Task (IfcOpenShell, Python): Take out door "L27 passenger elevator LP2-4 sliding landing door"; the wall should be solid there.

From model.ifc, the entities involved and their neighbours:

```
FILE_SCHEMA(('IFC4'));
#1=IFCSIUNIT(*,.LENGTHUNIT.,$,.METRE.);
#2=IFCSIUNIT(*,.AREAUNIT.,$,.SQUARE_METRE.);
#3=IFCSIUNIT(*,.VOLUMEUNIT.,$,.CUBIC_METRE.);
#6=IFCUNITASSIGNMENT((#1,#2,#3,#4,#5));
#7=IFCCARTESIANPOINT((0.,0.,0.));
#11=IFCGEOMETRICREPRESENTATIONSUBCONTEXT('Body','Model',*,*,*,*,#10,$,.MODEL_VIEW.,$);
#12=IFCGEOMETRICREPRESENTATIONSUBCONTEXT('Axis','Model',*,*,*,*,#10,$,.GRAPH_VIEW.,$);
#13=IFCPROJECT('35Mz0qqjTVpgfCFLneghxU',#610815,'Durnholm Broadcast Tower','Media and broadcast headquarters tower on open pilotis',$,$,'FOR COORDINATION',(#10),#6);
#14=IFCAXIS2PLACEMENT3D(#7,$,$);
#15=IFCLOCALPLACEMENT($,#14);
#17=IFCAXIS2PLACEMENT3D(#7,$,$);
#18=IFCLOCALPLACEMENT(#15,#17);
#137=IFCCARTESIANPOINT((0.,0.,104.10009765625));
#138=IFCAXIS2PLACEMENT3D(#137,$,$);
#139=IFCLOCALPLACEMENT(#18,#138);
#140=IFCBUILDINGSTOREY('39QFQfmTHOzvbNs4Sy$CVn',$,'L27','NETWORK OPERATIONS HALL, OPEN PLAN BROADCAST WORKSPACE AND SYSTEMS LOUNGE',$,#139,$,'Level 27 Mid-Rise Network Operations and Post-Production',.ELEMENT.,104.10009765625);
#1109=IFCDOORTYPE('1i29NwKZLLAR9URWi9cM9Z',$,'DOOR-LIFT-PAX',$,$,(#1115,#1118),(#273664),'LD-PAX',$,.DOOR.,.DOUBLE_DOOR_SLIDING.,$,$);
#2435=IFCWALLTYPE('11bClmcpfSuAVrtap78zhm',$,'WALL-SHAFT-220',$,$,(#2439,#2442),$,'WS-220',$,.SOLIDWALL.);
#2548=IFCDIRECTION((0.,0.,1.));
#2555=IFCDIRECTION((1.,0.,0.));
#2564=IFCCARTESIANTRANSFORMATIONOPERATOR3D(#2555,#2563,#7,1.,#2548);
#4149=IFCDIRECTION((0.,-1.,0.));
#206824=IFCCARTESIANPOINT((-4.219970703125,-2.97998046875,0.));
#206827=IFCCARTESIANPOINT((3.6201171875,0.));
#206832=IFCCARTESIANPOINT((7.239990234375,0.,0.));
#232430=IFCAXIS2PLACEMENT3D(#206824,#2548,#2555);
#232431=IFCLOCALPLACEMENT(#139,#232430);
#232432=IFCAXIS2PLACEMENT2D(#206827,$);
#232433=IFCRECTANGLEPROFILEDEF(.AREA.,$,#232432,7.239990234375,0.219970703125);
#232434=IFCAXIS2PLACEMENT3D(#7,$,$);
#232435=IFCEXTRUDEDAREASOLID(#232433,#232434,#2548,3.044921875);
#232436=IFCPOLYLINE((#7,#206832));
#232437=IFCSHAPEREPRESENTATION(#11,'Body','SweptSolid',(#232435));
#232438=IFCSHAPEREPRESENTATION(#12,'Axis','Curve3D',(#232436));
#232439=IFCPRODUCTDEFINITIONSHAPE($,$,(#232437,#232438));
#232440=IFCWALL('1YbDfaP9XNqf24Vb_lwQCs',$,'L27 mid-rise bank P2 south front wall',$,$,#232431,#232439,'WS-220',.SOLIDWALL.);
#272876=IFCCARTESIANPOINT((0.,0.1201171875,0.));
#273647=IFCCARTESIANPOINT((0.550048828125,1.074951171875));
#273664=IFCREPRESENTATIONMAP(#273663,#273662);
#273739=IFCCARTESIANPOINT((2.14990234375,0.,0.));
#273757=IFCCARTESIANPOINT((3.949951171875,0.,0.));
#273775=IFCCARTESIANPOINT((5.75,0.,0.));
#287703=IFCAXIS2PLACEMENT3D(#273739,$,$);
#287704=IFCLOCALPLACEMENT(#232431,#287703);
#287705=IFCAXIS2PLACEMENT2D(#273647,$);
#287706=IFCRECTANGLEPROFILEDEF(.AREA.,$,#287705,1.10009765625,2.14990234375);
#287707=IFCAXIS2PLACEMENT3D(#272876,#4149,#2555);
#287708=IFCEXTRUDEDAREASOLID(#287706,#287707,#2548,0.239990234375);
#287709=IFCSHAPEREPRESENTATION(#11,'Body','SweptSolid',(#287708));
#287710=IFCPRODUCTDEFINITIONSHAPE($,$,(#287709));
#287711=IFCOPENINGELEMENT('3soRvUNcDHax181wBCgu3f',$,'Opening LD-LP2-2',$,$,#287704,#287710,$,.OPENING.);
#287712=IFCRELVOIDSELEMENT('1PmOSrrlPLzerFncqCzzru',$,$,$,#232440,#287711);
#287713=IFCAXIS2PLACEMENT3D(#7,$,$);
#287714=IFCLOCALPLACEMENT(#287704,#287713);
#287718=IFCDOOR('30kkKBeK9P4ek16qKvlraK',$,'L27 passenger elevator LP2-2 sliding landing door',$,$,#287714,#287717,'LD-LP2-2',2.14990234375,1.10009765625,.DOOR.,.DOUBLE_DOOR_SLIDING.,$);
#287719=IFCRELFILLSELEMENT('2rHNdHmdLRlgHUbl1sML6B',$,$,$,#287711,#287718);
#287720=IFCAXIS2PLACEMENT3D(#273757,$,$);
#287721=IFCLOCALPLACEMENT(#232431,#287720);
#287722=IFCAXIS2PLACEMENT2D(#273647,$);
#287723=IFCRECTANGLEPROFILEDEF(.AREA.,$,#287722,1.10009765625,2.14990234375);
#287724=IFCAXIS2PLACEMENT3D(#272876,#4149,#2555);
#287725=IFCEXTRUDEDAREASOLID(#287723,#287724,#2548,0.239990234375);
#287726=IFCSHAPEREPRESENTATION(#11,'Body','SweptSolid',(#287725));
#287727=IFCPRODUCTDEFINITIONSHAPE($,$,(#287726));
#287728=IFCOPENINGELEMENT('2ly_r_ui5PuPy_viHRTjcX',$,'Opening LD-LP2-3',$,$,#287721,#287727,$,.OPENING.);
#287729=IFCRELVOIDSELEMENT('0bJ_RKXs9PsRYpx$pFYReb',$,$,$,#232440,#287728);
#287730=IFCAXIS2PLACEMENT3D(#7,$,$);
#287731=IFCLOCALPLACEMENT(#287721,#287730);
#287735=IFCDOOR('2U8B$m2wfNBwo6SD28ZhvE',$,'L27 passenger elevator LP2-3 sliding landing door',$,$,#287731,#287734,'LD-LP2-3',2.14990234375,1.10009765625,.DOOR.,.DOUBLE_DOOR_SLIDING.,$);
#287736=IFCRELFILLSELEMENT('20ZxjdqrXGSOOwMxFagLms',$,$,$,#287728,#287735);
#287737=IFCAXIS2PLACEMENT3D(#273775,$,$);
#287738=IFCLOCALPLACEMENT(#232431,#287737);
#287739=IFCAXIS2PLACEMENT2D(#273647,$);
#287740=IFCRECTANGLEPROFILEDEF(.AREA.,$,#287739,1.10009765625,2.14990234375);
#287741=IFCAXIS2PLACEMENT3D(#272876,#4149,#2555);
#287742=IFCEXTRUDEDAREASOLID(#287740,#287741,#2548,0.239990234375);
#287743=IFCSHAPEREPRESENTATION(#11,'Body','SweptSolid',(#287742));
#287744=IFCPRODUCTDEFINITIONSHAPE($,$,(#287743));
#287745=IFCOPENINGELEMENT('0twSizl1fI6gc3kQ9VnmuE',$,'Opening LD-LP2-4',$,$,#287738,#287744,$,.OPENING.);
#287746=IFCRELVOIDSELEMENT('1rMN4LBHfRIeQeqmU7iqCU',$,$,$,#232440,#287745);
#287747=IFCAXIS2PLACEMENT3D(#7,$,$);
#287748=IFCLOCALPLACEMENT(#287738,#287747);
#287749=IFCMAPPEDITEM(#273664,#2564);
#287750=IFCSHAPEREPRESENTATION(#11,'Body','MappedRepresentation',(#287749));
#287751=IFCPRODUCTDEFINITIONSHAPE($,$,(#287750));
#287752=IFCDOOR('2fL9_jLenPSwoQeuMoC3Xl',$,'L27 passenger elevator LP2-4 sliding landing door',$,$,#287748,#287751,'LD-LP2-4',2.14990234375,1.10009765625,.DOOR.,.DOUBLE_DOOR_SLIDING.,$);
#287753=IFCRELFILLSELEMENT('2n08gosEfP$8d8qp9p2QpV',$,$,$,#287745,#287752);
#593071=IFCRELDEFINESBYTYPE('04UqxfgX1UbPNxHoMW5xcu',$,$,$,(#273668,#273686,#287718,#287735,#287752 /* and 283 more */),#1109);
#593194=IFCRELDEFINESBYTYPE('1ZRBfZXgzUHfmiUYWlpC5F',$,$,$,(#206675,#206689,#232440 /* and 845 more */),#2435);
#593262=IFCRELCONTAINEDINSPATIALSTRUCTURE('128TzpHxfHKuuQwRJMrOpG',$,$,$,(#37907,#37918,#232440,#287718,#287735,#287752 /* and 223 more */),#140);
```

```python
import ifcopenshell
import ifcopenshell.api.feature
import ifcopenshell.api.root
import ifcopenshell.geom
import ifcopenshell.util.shape

model = ifcopenshell.open("model.ifc")
settings = ifcopenshell.geom.settings()


def volume(element):
    """Net volume in cubic metres, openings subtracted."""
    shape = ifcopenshell.geom.create_shape(settings, element)
    return ifcopenshell.util.shape.get_volume(shape.geometry)


door = model.by_guid("2fL9_jLenPSwoQeuMoC3Xl")
opening = door.FillsVoids[0].RelatingOpeningElement
wall = opening.VoidsElements[0].RelatingBuildingElement
before = volume(wall)

ifcopenshell.api.root.remove_product(model, product=door)
ifcopenshell.api.feature.remove_feature(model, feature=opening)

after = volume(wall)

print(f"wall volume {before:.3f} -> {after:.3f} m3")

model.write("model_edited.ifc")
```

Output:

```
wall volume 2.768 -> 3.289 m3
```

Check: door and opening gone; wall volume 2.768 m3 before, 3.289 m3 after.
